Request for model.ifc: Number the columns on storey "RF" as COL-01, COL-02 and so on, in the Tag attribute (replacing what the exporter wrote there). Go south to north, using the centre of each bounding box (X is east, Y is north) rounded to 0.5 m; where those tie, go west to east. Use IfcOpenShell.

First a look at what the model holds.

```python
import ifcopenshell
import ifcopenshell.util.element
import ifcopenshell.util.placement

model = ifcopenshell.open("model.ifc")
print(model.schema)
storey = next(s for s in model.by_type("IfcBuildingStorey") if s.Name == "RF")
columns = [e for e in ifcopenshell.util.element.get_decomposition(storey) if e.is_a("IfcColumn")]
for e in sorted(columns, key=lambda e: e.id()):
    origin = ifcopenshell.util.placement.get_local_placement(e.ObjectPlacement)[:3, 3]
    print(e.id(), e.Tag, e.Name, origin.round(2) + 0.0, sep=" | ")
```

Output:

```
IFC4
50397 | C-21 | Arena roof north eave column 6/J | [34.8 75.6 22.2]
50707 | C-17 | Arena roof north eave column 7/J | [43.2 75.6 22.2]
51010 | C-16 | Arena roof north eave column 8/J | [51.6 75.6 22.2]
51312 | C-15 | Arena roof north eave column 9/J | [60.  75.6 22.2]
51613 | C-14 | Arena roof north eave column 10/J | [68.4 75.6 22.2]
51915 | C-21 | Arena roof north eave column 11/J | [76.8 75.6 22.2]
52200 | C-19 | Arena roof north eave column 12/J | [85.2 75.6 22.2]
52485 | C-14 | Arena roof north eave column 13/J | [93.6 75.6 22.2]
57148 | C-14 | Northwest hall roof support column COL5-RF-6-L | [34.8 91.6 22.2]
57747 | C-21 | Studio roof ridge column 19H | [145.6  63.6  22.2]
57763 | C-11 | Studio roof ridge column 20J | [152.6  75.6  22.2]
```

```python
import ifcopenshell
import ifcopenshell.geom
import ifcopenshell.util.element
import ifcopenshell.util.shape

model = ifcopenshell.open("model.ifc")
settings = ifcopenshell.geom.settings()
settings.set("use-world-coords", True)


def centre(element):
    shape = ifcopenshell.geom.create_shape(settings, element)
    return ifcopenshell.util.shape.get_bbox_centroid(shape.geometry)


storey = next(s for s in model.by_type("IfcBuildingStorey") if s.Name == "RF")
columns = [e for e in ifcopenshell.util.element.get_decomposition(storey) if e.is_a("IfcColumn")]

# Insertion points can sit at a corner or the storey origin, so sort by the geometry (in metres).
centres = {e: centre(e) for e in columns}
columns.sort(key=lambda e: (round(centres[e][1] / 0.5), centres[e][0]))

for i, e in enumerate(columns, start=1):
    number = f"COL-{i:02d}"
    e.Tag = number
    print(e.id(), number)

model.write("model_edited.ifc")
```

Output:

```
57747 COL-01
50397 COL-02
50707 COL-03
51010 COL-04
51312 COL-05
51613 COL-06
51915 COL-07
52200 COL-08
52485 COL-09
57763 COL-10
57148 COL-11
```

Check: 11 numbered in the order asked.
